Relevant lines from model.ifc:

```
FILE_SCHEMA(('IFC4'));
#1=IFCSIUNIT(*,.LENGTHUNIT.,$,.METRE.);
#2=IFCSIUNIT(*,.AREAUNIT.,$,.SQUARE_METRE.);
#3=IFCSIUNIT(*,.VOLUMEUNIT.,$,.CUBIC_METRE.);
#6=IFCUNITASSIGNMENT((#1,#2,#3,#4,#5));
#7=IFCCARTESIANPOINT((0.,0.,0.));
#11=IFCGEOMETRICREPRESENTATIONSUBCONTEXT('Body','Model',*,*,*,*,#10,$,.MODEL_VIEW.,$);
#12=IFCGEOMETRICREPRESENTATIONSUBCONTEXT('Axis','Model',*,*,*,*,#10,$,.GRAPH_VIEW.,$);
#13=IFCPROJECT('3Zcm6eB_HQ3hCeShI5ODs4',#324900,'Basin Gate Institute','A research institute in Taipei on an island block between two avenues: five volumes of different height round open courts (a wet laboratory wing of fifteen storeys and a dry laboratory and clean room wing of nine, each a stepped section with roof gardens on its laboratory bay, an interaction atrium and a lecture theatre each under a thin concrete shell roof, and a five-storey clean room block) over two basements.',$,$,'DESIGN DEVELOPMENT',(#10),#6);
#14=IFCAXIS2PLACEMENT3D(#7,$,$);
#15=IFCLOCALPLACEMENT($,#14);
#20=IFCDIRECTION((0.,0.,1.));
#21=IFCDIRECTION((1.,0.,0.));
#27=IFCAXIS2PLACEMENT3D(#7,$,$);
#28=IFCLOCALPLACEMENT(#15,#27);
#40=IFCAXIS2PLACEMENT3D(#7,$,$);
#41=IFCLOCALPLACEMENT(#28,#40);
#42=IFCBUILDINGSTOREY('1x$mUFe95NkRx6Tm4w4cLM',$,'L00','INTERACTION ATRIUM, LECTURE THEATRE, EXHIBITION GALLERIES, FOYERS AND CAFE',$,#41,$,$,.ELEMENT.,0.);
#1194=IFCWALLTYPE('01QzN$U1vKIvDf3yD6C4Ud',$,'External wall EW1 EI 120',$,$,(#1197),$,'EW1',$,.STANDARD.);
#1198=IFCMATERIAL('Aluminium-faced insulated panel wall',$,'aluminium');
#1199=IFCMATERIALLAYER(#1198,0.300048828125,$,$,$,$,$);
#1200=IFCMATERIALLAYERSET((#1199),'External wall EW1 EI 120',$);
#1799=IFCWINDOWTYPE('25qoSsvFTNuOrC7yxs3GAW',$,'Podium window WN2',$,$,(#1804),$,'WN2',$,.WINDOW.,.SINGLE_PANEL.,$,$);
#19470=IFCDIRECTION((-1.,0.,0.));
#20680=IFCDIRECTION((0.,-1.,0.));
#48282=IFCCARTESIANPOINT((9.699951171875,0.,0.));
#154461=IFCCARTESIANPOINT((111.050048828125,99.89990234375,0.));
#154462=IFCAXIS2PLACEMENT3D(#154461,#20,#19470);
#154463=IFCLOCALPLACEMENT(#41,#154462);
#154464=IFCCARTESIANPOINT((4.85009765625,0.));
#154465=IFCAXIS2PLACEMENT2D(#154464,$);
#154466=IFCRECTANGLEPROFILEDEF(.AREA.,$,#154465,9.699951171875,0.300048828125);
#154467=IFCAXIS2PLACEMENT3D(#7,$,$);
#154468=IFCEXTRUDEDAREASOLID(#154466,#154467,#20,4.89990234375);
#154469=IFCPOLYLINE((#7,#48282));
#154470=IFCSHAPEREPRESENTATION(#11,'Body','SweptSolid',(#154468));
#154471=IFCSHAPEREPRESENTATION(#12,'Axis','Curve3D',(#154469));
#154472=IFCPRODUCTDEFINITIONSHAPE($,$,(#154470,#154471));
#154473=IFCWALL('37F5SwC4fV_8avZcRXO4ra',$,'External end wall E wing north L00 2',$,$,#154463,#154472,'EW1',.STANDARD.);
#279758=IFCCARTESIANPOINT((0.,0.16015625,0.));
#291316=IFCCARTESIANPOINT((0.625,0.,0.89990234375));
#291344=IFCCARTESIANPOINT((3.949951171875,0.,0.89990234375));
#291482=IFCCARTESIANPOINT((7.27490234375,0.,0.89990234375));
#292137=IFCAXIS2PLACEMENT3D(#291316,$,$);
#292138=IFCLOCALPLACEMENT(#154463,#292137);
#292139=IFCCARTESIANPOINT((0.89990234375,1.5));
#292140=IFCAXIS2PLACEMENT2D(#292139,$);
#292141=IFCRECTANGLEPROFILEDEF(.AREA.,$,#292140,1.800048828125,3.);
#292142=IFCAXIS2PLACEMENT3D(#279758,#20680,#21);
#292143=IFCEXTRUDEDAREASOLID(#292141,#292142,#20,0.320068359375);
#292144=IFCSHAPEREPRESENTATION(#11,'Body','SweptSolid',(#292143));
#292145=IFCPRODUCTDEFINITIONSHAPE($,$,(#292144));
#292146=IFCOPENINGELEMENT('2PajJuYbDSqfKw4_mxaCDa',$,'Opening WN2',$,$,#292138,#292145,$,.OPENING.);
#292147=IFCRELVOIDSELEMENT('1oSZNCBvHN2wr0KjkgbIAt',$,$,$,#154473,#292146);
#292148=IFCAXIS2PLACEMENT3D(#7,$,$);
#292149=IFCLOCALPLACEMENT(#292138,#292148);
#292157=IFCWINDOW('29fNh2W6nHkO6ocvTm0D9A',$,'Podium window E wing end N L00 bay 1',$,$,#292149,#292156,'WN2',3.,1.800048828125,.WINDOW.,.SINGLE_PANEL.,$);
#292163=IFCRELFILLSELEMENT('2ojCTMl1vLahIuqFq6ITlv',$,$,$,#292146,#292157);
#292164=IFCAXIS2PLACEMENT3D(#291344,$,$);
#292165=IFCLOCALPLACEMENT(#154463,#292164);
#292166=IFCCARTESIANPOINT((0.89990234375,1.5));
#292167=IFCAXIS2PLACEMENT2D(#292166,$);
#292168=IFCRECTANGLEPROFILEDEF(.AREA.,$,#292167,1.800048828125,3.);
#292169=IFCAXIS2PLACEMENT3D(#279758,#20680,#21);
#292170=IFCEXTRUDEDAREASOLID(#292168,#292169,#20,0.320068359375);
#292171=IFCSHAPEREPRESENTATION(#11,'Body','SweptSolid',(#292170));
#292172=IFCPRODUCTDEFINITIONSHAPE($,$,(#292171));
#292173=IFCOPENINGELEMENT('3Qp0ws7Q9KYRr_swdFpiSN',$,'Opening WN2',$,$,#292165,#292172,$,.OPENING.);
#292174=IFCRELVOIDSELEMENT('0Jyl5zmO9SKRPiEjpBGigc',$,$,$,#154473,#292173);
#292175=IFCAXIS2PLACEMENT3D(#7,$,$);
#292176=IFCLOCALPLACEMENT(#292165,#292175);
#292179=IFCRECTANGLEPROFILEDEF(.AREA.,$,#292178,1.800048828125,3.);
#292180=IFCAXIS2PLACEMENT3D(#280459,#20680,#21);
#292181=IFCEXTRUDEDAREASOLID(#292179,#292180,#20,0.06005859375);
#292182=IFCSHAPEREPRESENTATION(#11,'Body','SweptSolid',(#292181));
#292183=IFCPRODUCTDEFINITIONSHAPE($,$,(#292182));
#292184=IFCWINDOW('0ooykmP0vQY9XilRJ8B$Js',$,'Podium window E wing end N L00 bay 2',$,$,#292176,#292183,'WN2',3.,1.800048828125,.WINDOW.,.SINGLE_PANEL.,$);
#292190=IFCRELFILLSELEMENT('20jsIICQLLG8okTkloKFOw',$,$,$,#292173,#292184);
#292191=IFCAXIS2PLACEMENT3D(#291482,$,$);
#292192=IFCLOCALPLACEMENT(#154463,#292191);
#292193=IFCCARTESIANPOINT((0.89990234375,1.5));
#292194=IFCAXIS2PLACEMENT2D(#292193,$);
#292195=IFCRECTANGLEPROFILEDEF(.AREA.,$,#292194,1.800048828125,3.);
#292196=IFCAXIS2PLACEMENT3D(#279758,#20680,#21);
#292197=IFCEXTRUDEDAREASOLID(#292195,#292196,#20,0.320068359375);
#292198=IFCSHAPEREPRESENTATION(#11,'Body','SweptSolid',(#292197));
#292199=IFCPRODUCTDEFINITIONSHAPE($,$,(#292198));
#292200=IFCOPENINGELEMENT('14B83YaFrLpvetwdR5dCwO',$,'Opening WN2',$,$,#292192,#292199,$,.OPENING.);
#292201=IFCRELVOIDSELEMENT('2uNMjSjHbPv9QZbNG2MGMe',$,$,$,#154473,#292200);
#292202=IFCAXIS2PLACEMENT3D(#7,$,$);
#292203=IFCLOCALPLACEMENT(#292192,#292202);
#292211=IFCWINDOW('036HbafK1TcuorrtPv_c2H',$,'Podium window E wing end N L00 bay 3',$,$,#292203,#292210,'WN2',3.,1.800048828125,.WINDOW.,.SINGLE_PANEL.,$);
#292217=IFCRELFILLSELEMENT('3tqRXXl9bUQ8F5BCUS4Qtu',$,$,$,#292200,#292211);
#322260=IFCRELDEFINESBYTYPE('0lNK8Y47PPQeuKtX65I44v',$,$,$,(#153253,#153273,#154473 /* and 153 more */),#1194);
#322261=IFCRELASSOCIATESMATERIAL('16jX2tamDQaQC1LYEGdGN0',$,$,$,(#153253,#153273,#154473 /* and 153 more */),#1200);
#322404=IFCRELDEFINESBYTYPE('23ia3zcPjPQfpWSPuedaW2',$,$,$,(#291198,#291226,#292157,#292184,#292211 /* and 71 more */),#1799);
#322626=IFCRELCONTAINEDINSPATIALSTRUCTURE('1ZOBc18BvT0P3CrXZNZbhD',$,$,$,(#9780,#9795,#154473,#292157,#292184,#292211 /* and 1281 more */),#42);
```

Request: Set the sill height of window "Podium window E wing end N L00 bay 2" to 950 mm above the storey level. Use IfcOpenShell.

```python
import numpy as np
import ifcopenshell
import ifcopenshell.api.geometry
import ifcopenshell.geom
import ifcopenshell.util.element
import ifcopenshell.util.placement
import ifcopenshell.util.shape
import ifcopenshell.util.unit

model = ifcopenshell.open("model.ifc")
unit_scale = ifcopenshell.util.unit.calculate_unit_scale(model)

window = model.by_guid("0ooykmP0vQY9XilRJ8B$Js")
opening = window.FillsVoids[0].RelatingOpeningElement
storey = ifcopenshell.util.element.get_container(window, ifc_class="IfcBuildingStorey")
level = ifcopenshell.util.placement.get_local_placement(storey.ObjectPlacement)[2, 3]

# The opening's origin need not be at the sill, so measure its lowest point.
shape = ifcopenshell.geom.create_shape(ifcopenshell.geom.settings(), opening)
bottom = ifcopenshell.util.shape.get_shape_bottom_elevation(shape, shape.geometry) / unit_scale
dz = level + 0.95 / unit_scale - bottom

shift = np.array([0.0, 0.0, dz])
# The window is placed relative to its opening, so it follows when the opening moves.
matrix = ifcopenshell.util.placement.get_local_placement(opening.ObjectPlacement)
matrix[:3, 3] += shift
ifcopenshell.api.geometry.edit_object_placement(
    model, product=opening, matrix=matrix, is_si=False, should_transform_children=True
)

print(f"moved by {dz * unit_scale:+.3f} m")

model.write("model_v2.ifc")
```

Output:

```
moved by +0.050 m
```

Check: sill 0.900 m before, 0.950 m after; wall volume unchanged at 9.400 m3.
